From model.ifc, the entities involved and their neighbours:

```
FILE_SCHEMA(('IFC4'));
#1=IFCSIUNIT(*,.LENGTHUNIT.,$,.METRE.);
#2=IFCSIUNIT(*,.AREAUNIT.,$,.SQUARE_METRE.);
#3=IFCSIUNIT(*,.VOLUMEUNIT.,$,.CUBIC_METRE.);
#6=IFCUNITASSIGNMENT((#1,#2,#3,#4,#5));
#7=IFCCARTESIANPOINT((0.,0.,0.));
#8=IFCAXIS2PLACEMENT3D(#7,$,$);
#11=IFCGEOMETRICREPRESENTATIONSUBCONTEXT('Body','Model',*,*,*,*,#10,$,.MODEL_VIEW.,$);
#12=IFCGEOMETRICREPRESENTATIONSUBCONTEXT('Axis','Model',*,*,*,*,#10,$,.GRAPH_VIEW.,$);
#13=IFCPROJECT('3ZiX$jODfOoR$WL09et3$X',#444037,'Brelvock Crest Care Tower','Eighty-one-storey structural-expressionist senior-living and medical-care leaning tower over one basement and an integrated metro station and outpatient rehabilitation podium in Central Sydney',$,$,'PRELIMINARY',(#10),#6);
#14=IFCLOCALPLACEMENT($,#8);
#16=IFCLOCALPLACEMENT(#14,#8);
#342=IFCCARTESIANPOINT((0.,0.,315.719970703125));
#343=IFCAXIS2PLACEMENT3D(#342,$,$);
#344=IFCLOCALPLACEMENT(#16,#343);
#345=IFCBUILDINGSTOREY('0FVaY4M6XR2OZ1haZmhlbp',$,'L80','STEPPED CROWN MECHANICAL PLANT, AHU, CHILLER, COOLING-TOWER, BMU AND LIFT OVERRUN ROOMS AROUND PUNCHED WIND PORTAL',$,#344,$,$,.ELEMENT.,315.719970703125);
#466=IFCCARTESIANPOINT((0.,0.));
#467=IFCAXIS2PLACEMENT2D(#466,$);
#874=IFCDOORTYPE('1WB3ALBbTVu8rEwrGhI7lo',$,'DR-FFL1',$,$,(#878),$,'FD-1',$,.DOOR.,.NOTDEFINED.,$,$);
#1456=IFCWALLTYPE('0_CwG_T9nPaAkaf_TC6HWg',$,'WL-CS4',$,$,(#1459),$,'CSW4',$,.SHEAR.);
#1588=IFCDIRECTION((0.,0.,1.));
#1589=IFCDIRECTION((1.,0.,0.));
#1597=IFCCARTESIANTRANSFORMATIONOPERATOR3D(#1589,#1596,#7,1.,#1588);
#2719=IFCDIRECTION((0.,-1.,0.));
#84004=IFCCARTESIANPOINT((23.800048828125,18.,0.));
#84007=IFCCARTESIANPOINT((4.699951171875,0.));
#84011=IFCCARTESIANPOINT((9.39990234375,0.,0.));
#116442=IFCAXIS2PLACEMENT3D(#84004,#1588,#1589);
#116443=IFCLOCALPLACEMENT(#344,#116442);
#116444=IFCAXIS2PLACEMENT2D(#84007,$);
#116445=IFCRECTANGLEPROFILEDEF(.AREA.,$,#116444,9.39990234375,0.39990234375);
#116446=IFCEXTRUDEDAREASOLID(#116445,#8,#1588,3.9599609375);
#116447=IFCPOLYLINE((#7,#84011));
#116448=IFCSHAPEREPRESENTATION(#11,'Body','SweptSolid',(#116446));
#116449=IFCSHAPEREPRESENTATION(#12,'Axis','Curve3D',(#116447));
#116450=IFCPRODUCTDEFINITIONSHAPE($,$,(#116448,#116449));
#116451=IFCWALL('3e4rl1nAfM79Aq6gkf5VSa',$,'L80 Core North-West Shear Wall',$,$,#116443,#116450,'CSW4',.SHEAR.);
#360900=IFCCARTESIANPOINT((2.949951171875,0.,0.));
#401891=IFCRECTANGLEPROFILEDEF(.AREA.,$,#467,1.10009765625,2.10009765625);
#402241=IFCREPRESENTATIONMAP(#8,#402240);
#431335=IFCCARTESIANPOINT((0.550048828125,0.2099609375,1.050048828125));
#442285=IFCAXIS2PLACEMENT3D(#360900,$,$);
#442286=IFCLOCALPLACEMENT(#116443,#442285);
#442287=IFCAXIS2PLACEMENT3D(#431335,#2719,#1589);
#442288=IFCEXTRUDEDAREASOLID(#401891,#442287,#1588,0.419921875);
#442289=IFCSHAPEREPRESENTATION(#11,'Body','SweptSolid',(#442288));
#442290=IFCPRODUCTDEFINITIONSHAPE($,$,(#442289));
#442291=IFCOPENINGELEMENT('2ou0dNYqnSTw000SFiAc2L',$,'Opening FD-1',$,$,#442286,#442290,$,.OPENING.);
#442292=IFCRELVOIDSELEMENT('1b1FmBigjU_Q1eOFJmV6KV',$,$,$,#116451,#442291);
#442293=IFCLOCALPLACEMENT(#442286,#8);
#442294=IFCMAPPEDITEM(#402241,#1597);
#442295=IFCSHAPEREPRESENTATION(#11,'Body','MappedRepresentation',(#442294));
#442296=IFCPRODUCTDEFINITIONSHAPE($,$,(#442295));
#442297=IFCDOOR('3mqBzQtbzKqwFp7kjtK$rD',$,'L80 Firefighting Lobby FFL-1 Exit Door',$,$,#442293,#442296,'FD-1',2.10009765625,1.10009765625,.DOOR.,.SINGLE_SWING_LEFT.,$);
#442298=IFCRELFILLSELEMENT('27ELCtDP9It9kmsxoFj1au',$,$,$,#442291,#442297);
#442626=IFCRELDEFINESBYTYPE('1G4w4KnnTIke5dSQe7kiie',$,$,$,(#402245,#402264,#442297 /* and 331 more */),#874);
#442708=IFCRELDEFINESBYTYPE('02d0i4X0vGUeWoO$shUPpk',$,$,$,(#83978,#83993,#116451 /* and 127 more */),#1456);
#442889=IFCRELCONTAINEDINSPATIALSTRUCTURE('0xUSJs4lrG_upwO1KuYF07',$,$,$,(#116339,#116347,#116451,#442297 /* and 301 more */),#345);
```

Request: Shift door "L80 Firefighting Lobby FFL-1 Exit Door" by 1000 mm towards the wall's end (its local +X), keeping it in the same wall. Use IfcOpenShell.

```python
import ifcopenshell
import ifcopenshell.api.geometry
import ifcopenshell.util.placement
import ifcopenshell.util.unit

model = ifcopenshell.open("model.ifc")
unit_scale = ifcopenshell.util.unit.calculate_unit_scale(model)

door = model.by_id(442297)
opening = door.FillsVoids[0].RelatingOpeningElement
wall = opening.VoidsElements[0].RelatingBuildingElement

wall_matrix = ifcopenshell.util.placement.get_local_placement(wall.ObjectPlacement)
shift = wall_matrix[:3, 0] * 1 / unit_scale
before = ifcopenshell.util.placement.get_local_placement(door.ObjectPlacement)[:3, 3].copy()

# The door is placed relative to its opening, so it follows when the opening moves.
matrix = ifcopenshell.util.placement.get_local_placement(opening.ObjectPlacement)
matrix[:3, 3] += shift
ifcopenshell.api.geometry.edit_object_placement(
    model, product=opening, matrix=matrix, is_si=False, should_transform_children=True
)

after = ifcopenshell.util.placement.get_local_placement(door.ObjectPlacement)[:3, 3]
print("door moved by", (after - before).round(3) + 0.0)

model.write("model_updated.ifc")
```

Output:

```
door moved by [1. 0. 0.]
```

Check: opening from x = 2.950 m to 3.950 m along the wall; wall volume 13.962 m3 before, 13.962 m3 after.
